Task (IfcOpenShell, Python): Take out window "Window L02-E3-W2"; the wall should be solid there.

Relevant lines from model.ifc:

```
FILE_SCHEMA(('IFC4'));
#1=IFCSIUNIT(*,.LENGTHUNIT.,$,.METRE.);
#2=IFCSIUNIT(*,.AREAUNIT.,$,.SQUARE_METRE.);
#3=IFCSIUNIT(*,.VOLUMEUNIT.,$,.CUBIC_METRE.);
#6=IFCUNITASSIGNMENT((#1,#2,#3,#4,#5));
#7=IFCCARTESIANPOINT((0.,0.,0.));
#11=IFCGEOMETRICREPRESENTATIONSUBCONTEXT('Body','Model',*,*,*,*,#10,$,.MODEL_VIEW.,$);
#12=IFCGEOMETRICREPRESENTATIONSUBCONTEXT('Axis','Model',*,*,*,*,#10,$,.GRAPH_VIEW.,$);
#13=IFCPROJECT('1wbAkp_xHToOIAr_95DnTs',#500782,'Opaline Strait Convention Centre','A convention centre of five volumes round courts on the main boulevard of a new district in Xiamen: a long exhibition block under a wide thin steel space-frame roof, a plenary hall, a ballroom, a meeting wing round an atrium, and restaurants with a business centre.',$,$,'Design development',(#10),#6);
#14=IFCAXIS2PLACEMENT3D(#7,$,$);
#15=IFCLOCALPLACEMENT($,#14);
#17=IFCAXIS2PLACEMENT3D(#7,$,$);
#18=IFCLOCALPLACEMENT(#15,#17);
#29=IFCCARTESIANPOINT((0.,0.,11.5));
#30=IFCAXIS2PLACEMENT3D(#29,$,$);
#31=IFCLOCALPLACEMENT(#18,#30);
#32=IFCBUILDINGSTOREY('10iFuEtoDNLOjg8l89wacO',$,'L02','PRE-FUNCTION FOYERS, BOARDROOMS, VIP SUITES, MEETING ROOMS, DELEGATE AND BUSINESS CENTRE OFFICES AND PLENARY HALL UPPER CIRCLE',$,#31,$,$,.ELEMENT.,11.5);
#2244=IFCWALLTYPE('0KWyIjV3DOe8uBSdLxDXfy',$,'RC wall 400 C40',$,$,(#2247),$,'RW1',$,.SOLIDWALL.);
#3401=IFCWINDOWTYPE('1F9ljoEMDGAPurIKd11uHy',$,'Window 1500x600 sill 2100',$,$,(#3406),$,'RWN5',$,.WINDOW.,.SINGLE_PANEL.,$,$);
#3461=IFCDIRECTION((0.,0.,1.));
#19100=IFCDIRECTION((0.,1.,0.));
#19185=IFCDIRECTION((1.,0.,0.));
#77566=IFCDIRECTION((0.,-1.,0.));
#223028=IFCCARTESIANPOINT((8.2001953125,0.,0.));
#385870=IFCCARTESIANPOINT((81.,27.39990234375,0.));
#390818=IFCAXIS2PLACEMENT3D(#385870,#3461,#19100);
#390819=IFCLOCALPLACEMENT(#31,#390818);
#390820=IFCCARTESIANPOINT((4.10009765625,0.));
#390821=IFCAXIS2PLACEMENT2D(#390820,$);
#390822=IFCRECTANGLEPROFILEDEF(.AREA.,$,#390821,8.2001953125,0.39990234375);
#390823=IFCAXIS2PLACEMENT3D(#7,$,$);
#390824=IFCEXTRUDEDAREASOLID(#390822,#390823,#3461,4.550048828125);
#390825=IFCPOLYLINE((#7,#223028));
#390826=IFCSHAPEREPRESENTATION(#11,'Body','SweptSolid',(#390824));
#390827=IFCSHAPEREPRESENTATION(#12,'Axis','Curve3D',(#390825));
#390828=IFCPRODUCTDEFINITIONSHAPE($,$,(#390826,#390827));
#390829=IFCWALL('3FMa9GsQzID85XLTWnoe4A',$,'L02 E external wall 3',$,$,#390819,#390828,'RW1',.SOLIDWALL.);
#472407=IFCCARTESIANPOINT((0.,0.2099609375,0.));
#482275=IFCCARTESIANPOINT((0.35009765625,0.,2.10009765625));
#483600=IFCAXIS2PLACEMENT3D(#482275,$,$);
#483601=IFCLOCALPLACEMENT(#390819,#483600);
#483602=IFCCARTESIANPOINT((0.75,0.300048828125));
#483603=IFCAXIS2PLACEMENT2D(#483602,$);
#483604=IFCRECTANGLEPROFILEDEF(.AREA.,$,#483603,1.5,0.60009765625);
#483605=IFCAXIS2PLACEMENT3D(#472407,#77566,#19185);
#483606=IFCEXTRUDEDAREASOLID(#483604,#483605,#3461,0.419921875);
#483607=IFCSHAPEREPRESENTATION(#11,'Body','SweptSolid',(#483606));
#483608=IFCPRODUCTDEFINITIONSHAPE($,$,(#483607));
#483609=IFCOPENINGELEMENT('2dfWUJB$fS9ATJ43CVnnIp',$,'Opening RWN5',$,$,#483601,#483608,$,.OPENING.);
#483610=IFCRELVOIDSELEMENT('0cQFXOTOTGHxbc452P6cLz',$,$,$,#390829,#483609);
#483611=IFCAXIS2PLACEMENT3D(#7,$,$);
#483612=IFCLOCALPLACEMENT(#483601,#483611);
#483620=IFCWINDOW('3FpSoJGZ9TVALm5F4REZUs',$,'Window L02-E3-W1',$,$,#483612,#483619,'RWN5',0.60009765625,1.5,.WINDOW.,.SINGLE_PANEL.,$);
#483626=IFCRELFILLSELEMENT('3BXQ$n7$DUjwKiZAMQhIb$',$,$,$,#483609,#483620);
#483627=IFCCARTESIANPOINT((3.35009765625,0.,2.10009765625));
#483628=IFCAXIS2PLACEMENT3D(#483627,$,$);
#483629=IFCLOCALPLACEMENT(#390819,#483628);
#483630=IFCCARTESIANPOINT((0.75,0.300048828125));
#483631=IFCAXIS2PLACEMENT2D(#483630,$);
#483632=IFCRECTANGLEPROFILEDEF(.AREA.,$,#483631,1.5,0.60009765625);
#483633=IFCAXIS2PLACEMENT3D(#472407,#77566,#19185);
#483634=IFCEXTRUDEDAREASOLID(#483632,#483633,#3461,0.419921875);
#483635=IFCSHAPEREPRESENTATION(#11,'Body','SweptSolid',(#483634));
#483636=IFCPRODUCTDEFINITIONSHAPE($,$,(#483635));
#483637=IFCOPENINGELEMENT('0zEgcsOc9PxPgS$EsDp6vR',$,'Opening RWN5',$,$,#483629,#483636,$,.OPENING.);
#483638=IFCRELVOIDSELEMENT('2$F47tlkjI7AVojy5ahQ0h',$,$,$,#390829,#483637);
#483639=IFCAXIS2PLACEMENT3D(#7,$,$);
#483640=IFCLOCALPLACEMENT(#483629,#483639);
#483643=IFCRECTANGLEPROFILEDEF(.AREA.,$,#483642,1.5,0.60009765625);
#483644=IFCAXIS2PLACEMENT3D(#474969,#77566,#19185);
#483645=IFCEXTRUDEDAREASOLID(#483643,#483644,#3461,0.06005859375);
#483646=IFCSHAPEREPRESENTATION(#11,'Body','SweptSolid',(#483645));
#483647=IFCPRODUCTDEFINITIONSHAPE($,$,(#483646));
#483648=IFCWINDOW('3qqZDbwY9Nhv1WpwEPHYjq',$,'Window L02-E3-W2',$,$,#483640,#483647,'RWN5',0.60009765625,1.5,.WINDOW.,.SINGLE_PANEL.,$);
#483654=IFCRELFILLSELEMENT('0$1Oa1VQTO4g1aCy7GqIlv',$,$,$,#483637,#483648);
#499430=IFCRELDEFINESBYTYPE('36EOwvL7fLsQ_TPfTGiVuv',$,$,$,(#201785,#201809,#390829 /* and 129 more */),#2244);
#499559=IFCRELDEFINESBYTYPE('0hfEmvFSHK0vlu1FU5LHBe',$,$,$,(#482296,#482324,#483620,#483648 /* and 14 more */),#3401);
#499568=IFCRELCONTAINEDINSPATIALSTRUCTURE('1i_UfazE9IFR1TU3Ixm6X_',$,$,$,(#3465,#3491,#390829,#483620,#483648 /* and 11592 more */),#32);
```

```python
import ifcopenshell
import ifcopenshell.api.feature
import ifcopenshell.api.root
import ifcopenshell.geom
import ifcopenshell.util.shape

model = ifcopenshell.open("model.ifc")
settings = ifcopenshell.geom.settings()


def volume(element):
    """Net volume in cubic metres, openings subtracted."""
    shape = ifcopenshell.geom.create_shape(settings, element)
    return ifcopenshell.util.shape.get_volume(shape.geometry)


window = model.by_guid("3qqZDbwY9Nhv1WpwEPHYjq")
opening = window.FillsVoids[0].RelatingOpeningElement
wall = opening.VoidsElements[0].RelatingBuildingElement
before = volume(wall)

ifcopenshell.api.root.remove_product(model, product=window)
ifcopenshell.api.feature.remove_feature(model, feature=opening)

after = volume(wall)

print(f"wall volume {before:.3f} -> {after:.3f} m3")

model.write("model_v2.ifc")
```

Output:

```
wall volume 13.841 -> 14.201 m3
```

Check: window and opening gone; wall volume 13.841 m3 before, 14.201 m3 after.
